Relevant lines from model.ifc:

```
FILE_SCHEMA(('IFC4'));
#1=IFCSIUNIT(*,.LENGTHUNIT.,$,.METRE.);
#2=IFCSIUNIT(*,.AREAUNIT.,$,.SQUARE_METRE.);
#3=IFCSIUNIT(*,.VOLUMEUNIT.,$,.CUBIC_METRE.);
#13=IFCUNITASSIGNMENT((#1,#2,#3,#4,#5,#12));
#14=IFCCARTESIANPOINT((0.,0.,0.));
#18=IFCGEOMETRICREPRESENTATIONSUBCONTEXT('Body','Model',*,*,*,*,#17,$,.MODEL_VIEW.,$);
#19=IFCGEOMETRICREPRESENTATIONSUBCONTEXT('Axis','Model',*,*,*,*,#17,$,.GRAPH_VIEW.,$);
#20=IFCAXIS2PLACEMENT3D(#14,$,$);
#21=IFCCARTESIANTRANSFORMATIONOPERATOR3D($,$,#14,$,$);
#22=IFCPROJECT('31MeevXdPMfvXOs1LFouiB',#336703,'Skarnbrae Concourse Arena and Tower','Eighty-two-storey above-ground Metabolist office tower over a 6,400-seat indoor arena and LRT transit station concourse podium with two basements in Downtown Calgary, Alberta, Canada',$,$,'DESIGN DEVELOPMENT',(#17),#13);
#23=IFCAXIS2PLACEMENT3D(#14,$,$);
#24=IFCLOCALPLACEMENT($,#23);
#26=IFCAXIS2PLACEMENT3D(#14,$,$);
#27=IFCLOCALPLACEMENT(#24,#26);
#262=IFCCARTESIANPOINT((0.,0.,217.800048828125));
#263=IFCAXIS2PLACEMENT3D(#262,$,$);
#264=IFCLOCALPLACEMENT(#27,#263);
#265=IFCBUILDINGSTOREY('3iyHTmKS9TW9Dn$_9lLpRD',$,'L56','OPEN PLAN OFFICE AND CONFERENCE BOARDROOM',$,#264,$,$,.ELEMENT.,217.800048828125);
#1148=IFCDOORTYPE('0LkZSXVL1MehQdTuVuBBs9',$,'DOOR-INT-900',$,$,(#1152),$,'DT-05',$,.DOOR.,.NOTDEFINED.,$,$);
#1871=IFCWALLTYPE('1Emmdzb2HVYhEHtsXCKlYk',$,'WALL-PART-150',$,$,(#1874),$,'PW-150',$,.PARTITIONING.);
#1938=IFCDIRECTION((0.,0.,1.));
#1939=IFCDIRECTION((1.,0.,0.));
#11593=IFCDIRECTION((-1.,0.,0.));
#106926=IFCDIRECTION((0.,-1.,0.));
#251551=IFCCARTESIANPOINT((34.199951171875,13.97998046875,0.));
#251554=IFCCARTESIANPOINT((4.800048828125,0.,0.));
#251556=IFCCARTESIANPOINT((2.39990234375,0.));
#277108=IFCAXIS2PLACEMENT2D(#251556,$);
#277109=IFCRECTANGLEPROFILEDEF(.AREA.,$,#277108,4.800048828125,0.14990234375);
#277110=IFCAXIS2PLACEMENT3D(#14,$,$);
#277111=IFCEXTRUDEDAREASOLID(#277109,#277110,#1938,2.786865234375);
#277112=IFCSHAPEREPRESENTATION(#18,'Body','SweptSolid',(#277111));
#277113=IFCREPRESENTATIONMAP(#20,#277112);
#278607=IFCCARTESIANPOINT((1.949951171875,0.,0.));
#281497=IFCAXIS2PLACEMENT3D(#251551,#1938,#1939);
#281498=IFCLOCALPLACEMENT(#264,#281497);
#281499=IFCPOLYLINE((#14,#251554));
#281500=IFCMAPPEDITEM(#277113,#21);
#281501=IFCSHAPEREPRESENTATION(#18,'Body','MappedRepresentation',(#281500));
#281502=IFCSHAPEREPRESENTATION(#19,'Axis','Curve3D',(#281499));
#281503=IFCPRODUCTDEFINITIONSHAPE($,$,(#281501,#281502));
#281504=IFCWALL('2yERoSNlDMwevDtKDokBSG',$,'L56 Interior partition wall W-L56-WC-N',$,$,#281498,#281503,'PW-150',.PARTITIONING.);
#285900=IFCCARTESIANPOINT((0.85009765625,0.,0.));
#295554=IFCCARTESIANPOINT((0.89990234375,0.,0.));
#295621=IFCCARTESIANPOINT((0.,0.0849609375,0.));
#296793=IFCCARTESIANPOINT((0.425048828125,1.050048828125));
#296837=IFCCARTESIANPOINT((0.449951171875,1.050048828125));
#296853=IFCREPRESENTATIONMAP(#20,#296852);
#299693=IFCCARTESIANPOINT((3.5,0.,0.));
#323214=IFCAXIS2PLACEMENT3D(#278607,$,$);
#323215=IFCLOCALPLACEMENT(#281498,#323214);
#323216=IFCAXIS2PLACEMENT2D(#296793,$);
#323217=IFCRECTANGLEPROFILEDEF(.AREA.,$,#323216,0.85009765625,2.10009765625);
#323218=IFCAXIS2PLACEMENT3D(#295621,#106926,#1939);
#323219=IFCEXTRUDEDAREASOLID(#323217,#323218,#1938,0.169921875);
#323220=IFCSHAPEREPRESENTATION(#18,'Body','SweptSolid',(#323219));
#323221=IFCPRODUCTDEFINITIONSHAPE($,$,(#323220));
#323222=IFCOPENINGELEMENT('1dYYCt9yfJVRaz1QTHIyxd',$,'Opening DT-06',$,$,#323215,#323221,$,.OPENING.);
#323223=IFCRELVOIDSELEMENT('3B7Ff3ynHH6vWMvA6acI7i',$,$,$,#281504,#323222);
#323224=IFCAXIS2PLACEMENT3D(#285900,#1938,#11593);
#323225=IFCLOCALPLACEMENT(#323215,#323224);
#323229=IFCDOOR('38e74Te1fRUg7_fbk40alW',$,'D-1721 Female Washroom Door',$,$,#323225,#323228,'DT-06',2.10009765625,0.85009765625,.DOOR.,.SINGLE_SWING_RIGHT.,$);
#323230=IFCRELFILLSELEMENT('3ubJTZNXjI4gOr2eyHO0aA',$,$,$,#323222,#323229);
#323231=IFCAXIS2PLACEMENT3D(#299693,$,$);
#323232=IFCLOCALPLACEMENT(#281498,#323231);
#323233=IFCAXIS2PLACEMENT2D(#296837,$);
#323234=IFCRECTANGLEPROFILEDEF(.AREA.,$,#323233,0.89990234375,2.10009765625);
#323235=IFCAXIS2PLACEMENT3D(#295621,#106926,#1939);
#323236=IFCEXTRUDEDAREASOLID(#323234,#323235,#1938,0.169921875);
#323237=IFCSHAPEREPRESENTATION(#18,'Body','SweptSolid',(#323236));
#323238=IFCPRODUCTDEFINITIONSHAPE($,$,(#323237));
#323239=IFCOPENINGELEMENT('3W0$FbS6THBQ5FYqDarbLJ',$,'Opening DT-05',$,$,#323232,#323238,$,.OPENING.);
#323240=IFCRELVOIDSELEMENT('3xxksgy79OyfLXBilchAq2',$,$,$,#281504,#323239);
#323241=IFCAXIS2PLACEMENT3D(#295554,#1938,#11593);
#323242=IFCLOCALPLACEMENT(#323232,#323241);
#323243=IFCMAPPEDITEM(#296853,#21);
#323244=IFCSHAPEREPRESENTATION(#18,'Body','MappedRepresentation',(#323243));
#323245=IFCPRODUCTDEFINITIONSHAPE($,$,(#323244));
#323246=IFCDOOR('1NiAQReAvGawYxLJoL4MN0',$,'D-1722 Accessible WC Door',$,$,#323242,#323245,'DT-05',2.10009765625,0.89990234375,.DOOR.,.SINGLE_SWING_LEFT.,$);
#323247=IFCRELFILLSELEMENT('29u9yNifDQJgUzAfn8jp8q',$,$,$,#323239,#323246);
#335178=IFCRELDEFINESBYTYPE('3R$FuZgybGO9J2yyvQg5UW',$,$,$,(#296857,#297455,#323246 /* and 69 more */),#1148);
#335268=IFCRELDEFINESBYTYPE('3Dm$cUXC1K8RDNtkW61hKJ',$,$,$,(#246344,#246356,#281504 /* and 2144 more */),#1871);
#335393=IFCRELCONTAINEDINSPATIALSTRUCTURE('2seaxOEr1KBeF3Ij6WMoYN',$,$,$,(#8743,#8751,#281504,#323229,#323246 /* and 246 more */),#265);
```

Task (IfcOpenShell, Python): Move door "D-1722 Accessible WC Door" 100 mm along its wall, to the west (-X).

```python
import ifcopenshell
import ifcopenshell.api.geometry
import ifcopenshell.util.placement
import ifcopenshell.util.unit

model = ifcopenshell.open("model.ifc")
unit_scale = ifcopenshell.util.unit.calculate_unit_scale(model)

door = model.by_id(323246)
opening = door.FillsVoids[0].RelatingOpeningElement
wall = opening.VoidsElements[0].RelatingBuildingElement

wall_matrix = ifcopenshell.util.placement.get_local_placement(wall.ObjectPlacement)
shift = wall_matrix[:3, 0] * -0.1 / unit_scale
before = ifcopenshell.util.placement.get_local_placement(door.ObjectPlacement)[:3, 3].copy()

# The door is placed relative to its opening, so it follows when the opening moves.
matrix = ifcopenshell.util.placement.get_local_placement(opening.ObjectPlacement)
matrix[:3, 3] += shift
ifcopenshell.api.geometry.edit_object_placement(
    model, product=opening, matrix=matrix, is_si=False, should_transform_children=True
)

after = ifcopenshell.util.placement.get_local_placement(door.ObjectPlacement)[:3, 3]
print("door moved by", (after - before).round(3) + 0.0)

model.write("model_rev.ifc")
```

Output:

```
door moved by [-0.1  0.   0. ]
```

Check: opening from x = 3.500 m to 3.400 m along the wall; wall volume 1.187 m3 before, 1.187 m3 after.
